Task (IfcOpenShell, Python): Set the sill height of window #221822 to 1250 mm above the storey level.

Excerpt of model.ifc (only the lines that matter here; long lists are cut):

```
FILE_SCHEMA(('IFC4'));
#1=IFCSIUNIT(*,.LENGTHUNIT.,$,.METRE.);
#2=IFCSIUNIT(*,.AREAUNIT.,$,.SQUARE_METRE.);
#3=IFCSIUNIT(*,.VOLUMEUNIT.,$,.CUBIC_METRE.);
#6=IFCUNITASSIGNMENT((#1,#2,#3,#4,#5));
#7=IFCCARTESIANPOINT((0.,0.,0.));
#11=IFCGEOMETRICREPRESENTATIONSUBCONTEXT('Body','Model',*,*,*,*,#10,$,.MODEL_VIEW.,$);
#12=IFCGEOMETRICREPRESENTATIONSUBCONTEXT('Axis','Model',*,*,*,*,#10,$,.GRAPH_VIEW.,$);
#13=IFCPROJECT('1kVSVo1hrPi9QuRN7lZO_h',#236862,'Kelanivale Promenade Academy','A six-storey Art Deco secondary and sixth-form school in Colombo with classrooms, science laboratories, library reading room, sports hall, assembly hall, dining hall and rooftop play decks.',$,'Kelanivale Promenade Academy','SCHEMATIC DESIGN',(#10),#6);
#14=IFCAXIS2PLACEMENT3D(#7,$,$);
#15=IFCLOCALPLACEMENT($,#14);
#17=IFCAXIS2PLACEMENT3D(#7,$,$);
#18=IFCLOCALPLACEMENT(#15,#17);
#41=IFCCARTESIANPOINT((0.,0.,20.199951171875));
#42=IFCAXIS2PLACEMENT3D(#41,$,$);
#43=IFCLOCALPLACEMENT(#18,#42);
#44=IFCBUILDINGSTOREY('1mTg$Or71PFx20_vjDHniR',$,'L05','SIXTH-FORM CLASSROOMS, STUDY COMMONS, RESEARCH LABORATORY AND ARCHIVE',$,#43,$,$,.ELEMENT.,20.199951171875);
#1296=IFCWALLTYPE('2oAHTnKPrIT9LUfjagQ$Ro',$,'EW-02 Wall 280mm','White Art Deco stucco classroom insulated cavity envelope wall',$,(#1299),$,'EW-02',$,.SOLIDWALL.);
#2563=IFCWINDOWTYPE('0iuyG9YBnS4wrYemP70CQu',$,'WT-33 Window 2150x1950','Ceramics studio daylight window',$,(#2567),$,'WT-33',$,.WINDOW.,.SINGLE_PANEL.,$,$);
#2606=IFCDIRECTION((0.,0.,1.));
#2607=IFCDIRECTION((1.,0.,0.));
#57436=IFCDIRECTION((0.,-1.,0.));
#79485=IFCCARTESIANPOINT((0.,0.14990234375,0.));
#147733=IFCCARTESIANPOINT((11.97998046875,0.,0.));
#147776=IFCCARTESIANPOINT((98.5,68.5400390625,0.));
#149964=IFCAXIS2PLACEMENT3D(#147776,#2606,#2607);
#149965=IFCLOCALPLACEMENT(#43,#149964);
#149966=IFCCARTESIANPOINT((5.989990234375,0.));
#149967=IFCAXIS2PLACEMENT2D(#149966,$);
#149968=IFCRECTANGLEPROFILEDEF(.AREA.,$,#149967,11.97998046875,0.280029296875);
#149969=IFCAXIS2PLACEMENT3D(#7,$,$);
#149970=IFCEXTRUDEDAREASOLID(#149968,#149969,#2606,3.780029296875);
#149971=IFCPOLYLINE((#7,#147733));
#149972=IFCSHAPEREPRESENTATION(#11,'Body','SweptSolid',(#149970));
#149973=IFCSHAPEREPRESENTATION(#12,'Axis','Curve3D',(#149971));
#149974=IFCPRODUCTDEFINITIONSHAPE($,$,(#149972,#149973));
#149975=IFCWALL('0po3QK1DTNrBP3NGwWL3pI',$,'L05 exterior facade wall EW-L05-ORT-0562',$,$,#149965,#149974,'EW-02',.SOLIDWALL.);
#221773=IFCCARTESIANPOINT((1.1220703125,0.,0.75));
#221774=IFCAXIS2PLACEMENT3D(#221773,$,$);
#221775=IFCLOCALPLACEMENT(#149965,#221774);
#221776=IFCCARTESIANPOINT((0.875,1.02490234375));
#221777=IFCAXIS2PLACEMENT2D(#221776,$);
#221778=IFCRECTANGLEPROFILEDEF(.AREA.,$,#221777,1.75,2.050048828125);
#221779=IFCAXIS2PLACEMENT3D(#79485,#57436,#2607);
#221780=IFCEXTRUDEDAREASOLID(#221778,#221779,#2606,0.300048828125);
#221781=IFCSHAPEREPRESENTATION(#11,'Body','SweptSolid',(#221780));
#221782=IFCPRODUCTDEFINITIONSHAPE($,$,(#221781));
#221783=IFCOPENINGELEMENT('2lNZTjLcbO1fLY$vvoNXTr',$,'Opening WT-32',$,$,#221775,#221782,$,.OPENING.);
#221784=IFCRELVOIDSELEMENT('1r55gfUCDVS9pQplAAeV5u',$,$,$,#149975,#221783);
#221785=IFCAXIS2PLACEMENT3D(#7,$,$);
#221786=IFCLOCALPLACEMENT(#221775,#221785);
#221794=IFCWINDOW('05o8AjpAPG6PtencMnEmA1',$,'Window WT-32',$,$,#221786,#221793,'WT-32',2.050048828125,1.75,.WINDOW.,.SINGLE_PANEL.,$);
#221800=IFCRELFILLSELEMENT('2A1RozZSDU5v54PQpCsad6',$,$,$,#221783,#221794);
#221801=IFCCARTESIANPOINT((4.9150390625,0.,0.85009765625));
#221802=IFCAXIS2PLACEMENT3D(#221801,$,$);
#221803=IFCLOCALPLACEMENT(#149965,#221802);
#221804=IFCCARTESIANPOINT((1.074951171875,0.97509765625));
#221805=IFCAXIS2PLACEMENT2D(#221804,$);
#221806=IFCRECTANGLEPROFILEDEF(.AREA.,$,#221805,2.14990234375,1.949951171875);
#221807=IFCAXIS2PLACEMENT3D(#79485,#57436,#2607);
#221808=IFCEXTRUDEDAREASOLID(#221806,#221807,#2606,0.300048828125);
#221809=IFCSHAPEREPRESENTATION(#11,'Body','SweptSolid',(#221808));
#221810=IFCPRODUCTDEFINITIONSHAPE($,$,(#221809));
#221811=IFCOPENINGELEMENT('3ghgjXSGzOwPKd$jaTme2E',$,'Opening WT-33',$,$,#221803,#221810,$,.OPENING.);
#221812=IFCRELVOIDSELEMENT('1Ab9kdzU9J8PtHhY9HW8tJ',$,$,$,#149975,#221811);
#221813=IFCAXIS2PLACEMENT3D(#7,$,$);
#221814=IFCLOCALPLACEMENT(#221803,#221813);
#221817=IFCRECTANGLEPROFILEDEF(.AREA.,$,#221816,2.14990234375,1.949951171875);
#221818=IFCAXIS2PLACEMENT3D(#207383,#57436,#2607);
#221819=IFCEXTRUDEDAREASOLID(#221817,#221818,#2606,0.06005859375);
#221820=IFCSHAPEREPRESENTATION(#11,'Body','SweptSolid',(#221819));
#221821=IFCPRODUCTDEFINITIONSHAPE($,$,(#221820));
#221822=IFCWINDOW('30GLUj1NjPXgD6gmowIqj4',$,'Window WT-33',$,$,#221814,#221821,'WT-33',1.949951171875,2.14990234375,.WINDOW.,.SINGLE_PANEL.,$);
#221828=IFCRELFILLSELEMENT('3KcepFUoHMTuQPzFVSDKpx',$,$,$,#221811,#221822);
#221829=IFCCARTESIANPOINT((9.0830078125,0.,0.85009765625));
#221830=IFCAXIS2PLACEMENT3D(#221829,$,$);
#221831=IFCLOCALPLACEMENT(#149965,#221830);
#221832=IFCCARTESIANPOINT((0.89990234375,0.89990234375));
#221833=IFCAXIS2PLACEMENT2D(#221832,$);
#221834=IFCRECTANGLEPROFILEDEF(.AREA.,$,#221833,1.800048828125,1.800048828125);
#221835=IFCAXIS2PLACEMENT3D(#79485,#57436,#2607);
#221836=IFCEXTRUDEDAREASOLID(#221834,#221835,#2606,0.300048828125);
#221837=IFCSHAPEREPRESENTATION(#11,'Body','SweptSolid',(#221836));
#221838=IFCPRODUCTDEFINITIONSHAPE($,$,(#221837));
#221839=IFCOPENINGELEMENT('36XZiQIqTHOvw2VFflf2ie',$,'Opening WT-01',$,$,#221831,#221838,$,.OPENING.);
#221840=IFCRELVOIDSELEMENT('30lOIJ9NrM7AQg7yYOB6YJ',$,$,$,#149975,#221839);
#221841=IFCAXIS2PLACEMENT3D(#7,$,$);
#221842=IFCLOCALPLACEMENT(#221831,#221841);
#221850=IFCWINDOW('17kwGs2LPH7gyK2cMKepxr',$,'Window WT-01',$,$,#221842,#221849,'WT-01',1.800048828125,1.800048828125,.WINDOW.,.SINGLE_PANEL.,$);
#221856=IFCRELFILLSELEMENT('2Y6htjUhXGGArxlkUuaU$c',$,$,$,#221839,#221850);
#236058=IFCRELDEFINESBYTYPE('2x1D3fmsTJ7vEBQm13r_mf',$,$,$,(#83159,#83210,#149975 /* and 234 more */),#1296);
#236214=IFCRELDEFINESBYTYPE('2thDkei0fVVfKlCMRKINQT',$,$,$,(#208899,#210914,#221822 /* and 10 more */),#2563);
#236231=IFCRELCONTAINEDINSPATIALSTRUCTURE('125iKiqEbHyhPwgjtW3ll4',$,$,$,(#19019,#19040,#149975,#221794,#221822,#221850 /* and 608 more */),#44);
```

```python
import numpy as np
import ifcopenshell
import ifcopenshell.api.geometry
import ifcopenshell.geom
import ifcopenshell.util.element
import ifcopenshell.util.placement
import ifcopenshell.util.shape
import ifcopenshell.util.unit

model = ifcopenshell.open("model.ifc")
unit_scale = ifcopenshell.util.unit.calculate_unit_scale(model)

window = model.by_id(221822)
opening = window.FillsVoids[0].RelatingOpeningElement
storey = ifcopenshell.util.element.get_container(window, ifc_class="IfcBuildingStorey")
level = ifcopenshell.util.placement.get_local_placement(storey.ObjectPlacement)[2, 3]

# The opening's origin need not be at the sill, so measure its lowest point.
shape = ifcopenshell.geom.create_shape(ifcopenshell.geom.settings(), opening)
bottom = ifcopenshell.util.shape.get_shape_bottom_elevation(shape, shape.geometry) / unit_scale
dz = level + 1.25 - bottom

shift = np.array([0.0, 0.0, dz])
# The window is placed relative to its opening, so it follows when the opening moves.
matrix = ifcopenshell.util.placement.get_local_placement(opening.ObjectPlacement)
matrix[:3, 3] += shift
ifcopenshell.api.geometry.edit_object_placement(
    model, product=opening, matrix=matrix, is_si=False, should_transform_children=True
)

print(f"moved by {dz * unit_scale:+.3f} m")

model.write("model_rev.ifc")
```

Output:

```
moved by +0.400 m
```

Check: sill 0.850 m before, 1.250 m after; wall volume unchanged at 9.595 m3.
